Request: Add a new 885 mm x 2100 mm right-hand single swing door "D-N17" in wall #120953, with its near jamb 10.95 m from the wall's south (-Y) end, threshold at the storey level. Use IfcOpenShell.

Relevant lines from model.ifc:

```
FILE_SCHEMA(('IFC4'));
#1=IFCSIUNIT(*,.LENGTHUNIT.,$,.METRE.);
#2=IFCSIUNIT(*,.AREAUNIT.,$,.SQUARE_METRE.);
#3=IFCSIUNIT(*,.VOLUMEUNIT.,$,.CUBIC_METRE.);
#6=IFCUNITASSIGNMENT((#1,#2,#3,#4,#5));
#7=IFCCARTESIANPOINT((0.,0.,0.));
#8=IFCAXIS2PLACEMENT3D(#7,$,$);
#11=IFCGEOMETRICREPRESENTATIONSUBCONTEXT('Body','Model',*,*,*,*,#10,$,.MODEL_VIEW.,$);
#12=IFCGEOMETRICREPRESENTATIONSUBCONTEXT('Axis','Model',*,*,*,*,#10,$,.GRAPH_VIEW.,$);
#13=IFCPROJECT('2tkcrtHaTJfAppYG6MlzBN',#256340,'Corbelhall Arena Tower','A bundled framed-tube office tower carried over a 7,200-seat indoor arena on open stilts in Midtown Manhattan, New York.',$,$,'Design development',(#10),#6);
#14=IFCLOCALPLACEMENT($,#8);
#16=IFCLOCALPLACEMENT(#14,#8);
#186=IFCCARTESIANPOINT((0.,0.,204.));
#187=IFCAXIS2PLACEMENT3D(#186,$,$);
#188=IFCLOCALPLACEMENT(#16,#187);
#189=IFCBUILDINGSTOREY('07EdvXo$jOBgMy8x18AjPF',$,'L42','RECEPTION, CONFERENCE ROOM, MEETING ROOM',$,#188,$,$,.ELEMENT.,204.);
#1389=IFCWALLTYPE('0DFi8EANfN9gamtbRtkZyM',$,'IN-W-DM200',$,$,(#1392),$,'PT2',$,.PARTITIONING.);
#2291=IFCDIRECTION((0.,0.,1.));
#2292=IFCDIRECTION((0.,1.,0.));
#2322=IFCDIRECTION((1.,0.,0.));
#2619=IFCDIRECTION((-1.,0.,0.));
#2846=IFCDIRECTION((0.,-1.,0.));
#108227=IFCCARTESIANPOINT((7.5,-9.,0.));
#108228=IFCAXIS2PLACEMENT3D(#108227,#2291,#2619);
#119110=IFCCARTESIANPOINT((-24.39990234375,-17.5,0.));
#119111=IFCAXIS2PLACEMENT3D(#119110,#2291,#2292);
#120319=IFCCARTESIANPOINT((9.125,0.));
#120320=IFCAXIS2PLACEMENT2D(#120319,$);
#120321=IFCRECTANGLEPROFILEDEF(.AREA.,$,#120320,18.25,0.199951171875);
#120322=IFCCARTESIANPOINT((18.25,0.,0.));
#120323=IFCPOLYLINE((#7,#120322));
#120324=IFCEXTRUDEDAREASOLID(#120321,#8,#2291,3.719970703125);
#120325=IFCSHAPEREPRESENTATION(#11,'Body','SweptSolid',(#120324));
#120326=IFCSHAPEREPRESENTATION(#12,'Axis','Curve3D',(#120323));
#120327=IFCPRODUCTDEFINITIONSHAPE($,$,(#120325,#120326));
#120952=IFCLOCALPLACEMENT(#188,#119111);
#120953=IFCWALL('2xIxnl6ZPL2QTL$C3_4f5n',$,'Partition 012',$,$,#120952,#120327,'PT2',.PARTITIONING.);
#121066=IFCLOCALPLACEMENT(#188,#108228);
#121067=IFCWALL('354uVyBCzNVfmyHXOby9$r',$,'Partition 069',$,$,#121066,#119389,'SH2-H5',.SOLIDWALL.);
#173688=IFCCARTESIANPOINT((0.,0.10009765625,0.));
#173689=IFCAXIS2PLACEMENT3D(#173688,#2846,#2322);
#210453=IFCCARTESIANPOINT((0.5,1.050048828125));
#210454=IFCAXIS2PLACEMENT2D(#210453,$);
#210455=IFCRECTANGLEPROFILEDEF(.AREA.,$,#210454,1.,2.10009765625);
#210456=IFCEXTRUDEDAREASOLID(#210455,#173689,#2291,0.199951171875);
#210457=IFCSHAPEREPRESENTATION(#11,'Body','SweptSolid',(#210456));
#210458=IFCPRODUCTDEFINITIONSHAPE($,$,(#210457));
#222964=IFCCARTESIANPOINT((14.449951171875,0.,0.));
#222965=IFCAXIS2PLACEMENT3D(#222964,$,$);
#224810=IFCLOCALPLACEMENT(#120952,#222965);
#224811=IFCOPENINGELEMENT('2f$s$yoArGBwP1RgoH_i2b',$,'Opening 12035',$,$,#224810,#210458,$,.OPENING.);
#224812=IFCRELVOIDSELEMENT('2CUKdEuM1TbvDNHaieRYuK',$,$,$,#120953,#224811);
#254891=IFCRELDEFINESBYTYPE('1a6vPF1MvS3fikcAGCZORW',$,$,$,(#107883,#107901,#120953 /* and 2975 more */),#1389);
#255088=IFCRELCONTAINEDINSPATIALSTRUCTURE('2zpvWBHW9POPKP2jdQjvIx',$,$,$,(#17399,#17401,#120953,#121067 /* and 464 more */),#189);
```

```python
import numpy as np
import ifcopenshell
import ifcopenshell.api.feature
import ifcopenshell.api.geometry
import ifcopenshell.api.root
import ifcopenshell.api.spatial
import ifcopenshell.geom
import ifcopenshell.util.element
import ifcopenshell.util.placement
import ifcopenshell.util.representation
import ifcopenshell.util.shape
import ifcopenshell.util.unit

model = ifcopenshell.open("model.ifc")
unit_scale = ifcopenshell.util.unit.calculate_unit_scale(model)
settings = ifcopenshell.geom.settings()


def volume(element):
    """Net volume in cubic metres, openings subtracted."""
    shape = ifcopenshell.geom.create_shape(settings, element)
    return ifcopenshell.util.shape.get_volume(shape.geometry)


wall = model.by_guid("2xIxnl6ZPL2QTL$C3_4f5n")
storey = ifcopenshell.util.element.get_container(wall, ifc_class="IfcBuildingStorey")
context = ifcopenshell.util.representation.get_context(model, "Model", "Body", "MODEL_VIEW")
before = volume(wall)

width, height, from_end, sill = 0.885, 2.1, 10.95, 0.0  # metres

# The wall runs along its own X axis, and the end named is its -X end.
wall_shape = ifcopenshell.geom.create_shape(settings, wall)
x, y, z = ifcopenshell.util.shape.get_vertices(wall_shape.geometry).T
start = x.min() + from_end
face, thickness = float(y.min()), float(y.max() - y.min())
wall_matrix = ifcopenshell.util.placement.get_local_placement(wall.ObjectPlacement)
level = ifcopenshell.util.placement.get_local_placement(storey.ObjectPlacement)[2, 3]


def in_wall(x, y):
    """Placement at x, y metres in the wall's axes, at sill height."""
    matrix = wall_matrix.copy()
    matrix[:, 3] = wall_matrix @ np.array([x / unit_scale, y / unit_scale, 0.0, 1.0])
    matrix[2, 3] = level + sill / unit_scale
    return matrix


# Opening: a box that overshoots both wall faces by 50 mm.
opening = ifcopenshell.api.root.create_entity(model, ifc_class="IfcOpeningElement", predefined_type="OPENING")
box = ifcopenshell.api.geometry.add_wall_representation(
    model, context=context, length=width, height=height, thickness=thickness + 0.1
)
ifcopenshell.api.geometry.assign_representation(model, product=opening, representation=box)
ifcopenshell.api.geometry.edit_object_placement(model, product=opening, matrix=in_wall(start, face - 0.05), is_si=False)
ifcopenshell.api.feature.add_feature(model, feature=opening, element=wall)

door = ifcopenshell.api.root.create_entity(model, ifc_class="IfcDoor", name="D-N17", predefined_type="DOOR")
door.OverallWidth, door.OverallHeight = width / unit_scale, height / unit_scale
door.OperationType = "SINGLE_SWING_RIGHT"
body = ifcopenshell.api.geometry.add_door_representation(
    model,
    context=context,
    overall_width=door.OverallWidth,
    overall_height=door.OverallHeight,
    operation_type="SINGLE_SWING_RIGHT",
    lining_properties={"LiningDepth": thickness / unit_scale, "ThresholdDepth": thickness / unit_scale},
)
ifcopenshell.api.geometry.assign_representation(model, product=door, representation=body)
ifcopenshell.api.spatial.assign_container(model, products=[door], relating_structure=storey)
ifcopenshell.api.feature.add_filling(model, opening=opening, element=door)

# The lining spans the wall, so the door starts at the wall face.
ifcopenshell.api.geometry.edit_object_placement(model, product=door, matrix=in_wall(start, face), is_si=False)

after = volume(wall)

print(f"wall volume {before:.3f} -> {after:.3f} m3")

model.write("model_updated.ifc")
```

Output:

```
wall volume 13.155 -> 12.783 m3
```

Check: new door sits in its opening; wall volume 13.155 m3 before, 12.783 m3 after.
